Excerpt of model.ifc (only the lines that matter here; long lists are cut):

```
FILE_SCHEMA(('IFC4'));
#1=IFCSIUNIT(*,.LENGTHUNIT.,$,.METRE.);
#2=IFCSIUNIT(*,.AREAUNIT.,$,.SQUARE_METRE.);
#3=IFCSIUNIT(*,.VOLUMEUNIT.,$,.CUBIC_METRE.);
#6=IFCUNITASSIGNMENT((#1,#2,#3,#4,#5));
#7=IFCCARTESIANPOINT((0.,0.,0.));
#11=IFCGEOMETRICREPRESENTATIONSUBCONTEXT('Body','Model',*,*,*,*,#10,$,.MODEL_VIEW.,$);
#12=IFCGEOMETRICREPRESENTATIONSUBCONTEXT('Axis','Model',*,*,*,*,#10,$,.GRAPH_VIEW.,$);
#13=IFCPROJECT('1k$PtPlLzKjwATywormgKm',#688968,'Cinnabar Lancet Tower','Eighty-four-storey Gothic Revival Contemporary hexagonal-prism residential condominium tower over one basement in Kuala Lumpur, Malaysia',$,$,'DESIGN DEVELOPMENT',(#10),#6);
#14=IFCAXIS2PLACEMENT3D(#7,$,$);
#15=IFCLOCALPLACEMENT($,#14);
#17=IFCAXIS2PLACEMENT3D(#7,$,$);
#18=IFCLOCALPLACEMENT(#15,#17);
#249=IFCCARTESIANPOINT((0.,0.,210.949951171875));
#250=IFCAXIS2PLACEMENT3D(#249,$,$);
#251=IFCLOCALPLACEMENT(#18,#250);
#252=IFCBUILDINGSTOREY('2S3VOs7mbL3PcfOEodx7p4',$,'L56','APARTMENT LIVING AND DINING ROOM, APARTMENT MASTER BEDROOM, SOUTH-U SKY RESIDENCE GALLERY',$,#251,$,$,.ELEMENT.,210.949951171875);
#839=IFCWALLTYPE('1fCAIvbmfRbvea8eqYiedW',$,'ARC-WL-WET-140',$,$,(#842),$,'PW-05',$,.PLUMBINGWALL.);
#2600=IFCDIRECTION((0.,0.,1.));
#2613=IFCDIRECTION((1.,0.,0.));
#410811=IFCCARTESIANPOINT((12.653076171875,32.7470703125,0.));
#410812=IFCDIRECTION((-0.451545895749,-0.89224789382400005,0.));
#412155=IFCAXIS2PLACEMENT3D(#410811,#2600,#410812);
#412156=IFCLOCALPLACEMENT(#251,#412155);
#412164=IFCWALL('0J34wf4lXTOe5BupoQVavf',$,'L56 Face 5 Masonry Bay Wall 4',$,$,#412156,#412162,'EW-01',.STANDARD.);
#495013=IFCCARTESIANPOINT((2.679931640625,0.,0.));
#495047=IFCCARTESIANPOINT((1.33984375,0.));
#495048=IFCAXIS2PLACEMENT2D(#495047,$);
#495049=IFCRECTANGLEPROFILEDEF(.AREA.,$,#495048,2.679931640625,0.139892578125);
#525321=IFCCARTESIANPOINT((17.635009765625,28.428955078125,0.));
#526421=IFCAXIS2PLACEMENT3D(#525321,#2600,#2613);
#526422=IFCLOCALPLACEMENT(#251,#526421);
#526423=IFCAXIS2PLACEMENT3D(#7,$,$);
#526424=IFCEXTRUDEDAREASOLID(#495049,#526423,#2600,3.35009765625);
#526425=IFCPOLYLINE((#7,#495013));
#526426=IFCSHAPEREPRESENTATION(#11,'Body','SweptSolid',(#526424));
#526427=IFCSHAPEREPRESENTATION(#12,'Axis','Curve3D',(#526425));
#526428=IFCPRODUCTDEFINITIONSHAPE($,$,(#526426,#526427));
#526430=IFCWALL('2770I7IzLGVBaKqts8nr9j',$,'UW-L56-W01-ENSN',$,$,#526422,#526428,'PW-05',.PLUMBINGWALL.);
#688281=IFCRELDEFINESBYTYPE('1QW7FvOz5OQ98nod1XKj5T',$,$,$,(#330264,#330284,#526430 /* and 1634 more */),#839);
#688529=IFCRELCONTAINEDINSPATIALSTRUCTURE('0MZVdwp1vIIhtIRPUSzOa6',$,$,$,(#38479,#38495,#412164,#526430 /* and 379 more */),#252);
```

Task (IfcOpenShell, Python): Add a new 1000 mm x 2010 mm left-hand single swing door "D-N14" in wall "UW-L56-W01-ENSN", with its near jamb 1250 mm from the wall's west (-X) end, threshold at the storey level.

```python
import numpy as np
import ifcopenshell
import ifcopenshell.api.feature
import ifcopenshell.api.geometry
import ifcopenshell.api.root
import ifcopenshell.api.spatial
import ifcopenshell.geom
import ifcopenshell.util.element
import ifcopenshell.util.placement
import ifcopenshell.util.representation
import ifcopenshell.util.shape
import ifcopenshell.util.unit

model = ifcopenshell.open("model.ifc")
unit_scale = ifcopenshell.util.unit.calculate_unit_scale(model)
settings = ifcopenshell.geom.settings()


def volume(element):
    """Net volume in cubic metres, openings subtracted."""
    shape = ifcopenshell.geom.create_shape(settings, element)
    return ifcopenshell.util.shape.get_volume(shape.geometry)


wall = model.by_guid("2770I7IzLGVBaKqts8nr9j")
storey = ifcopenshell.util.element.get_container(wall, ifc_class="IfcBuildingStorey")
context = ifcopenshell.util.representation.get_context(model, "Model", "Body", "MODEL_VIEW")
before = volume(wall)

width, height, from_end, sill = 1, 2.01, 1.25, 0.0  # metres

# The wall runs along its own X axis, and the end named is its -X end.
wall_shape = ifcopenshell.geom.create_shape(settings, wall)
x, y, z = ifcopenshell.util.shape.get_vertices(wall_shape.geometry).T
start = x.min() + from_end
face, thickness = float(y.min()), float(y.max() - y.min())
wall_matrix = ifcopenshell.util.placement.get_local_placement(wall.ObjectPlacement)
level = ifcopenshell.util.placement.get_local_placement(storey.ObjectPlacement)[2, 3]


def in_wall(x, y):
    """Placement at x, y metres in the wall's axes, at sill height."""
    matrix = wall_matrix.copy()
    matrix[:, 3] = wall_matrix @ np.array([x / unit_scale, y / unit_scale, 0.0, 1.0])
    matrix[2, 3] = level + sill / unit_scale
    return matrix


# Opening: a box that overshoots both wall faces by 50 mm.
opening = ifcopenshell.api.root.create_entity(model, ifc_class="IfcOpeningElement", predefined_type="OPENING")
box = ifcopenshell.api.geometry.add_wall_representation(
    model, context=context, length=width, height=height, thickness=thickness + 0.1
)
ifcopenshell.api.geometry.assign_representation(model, product=opening, representation=box)
ifcopenshell.api.geometry.edit_object_placement(model, product=opening, matrix=in_wall(start, face - 0.05), is_si=False)
ifcopenshell.api.feature.add_feature(model, feature=opening, element=wall)

door = ifcopenshell.api.root.create_entity(model, ifc_class="IfcDoor", name="D-N14", predefined_type="DOOR")
door.OverallWidth, door.OverallHeight = width / unit_scale, height / unit_scale
door.OperationType = "SINGLE_SWING_LEFT"
body = ifcopenshell.api.geometry.add_door_representation(
    model,
    context=context,
    overall_width=door.OverallWidth,
    overall_height=door.OverallHeight,
    operation_type="SINGLE_SWING_LEFT",
    lining_properties={"LiningDepth": thickness / unit_scale, "ThresholdDepth": thickness / unit_scale},
)
ifcopenshell.api.geometry.assign_representation(model, product=door, representation=body)
ifcopenshell.api.spatial.assign_container(model, products=[door], relating_structure=storey)
ifcopenshell.api.feature.add_filling(model, opening=opening, element=door)

# The lining spans the wall, so the door starts at the wall face.
ifcopenshell.api.geometry.edit_object_placement(model, product=door, matrix=in_wall(start, face), is_si=False)

after = volume(wall)

print(f"wall volume {before:.3f} -> {after:.3f} m3")

model.write("model_rev.ifc")
```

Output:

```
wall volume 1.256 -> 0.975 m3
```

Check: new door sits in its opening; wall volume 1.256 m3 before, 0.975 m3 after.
